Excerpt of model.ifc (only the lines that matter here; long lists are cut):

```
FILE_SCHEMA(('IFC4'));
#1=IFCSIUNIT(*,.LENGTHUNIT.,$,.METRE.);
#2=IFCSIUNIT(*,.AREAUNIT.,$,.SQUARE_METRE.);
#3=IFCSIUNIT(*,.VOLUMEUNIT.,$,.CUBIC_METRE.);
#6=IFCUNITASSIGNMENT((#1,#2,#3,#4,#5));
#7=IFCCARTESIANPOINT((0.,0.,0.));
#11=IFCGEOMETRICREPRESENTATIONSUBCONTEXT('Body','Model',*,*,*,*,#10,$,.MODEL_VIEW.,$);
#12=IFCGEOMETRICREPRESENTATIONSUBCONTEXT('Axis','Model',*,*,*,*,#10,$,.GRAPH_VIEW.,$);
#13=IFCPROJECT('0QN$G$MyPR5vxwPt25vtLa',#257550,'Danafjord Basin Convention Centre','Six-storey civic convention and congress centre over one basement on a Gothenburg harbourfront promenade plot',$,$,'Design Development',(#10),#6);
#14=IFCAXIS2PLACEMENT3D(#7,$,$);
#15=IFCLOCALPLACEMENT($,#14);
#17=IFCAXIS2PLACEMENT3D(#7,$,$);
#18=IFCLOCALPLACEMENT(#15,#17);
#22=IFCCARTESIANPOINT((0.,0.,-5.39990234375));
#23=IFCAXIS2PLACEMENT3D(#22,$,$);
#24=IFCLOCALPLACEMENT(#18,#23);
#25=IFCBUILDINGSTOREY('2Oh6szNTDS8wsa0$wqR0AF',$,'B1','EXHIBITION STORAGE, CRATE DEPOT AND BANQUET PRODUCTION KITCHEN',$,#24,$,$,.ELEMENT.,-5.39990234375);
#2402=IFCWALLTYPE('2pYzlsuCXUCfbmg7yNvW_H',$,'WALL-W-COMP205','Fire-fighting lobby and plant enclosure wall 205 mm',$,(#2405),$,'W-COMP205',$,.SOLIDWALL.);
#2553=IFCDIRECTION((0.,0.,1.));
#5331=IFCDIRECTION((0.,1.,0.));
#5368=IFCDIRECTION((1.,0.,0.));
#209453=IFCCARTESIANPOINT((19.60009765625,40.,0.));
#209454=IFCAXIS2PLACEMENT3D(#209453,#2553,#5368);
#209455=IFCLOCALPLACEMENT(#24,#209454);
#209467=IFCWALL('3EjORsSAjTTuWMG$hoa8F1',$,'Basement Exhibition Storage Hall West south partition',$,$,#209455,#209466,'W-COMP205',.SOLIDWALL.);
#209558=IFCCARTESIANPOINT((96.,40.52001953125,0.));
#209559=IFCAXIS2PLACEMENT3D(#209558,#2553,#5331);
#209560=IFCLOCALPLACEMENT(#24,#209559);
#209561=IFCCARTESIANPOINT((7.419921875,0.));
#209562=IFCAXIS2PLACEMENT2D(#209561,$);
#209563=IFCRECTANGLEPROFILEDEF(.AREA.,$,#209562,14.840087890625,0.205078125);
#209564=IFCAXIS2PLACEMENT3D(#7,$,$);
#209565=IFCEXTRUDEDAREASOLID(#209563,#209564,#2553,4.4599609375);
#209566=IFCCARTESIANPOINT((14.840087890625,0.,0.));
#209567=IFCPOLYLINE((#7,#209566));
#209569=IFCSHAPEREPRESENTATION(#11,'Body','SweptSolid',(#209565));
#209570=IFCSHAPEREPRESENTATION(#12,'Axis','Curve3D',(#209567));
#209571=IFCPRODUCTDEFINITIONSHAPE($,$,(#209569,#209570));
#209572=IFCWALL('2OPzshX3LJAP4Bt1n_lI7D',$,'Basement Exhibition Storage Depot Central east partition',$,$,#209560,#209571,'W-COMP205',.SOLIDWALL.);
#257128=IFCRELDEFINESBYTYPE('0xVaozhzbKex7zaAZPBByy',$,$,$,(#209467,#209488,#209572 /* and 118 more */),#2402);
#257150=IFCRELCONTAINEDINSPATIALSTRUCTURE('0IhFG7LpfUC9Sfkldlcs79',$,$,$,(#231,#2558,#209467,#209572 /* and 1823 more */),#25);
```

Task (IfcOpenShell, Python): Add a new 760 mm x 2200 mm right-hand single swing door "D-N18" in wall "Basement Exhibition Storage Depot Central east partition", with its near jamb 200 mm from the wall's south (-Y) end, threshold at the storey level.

```python
import numpy as np
import ifcopenshell
import ifcopenshell.api.feature
import ifcopenshell.api.geometry
import ifcopenshell.api.root
import ifcopenshell.api.spatial
import ifcopenshell.geom
import ifcopenshell.util.element
import ifcopenshell.util.placement
import ifcopenshell.util.representation
import ifcopenshell.util.shape
import ifcopenshell.util.unit

model = ifcopenshell.open("model.ifc")
unit_scale = ifcopenshell.util.unit.calculate_unit_scale(model)
settings = ifcopenshell.geom.settings()


def volume(element):
    """Net volume in cubic metres, openings subtracted."""
    shape = ifcopenshell.geom.create_shape(settings, element)
    return ifcopenshell.util.shape.get_volume(shape.geometry)


wall = model.by_guid("2OPzshX3LJAP4Bt1n_lI7D")
storey = ifcopenshell.util.element.get_container(wall, ifc_class="IfcBuildingStorey")
context = ifcopenshell.util.representation.get_context(model, "Model", "Body", "MODEL_VIEW")
before = volume(wall)

width, height, from_end, sill = 0.76, 2.2, 0.2, 0.0  # metres

# The wall runs along its own X axis, and the end named is its -X end.
wall_shape = ifcopenshell.geom.create_shape(settings, wall)
x, y, z = ifcopenshell.util.shape.get_vertices(wall_shape.geometry).T
start = x.min() + from_end
face, thickness = float(y.min()), float(y.max() - y.min())
wall_matrix = ifcopenshell.util.placement.get_local_placement(wall.ObjectPlacement)
level = ifcopenshell.util.placement.get_local_placement(storey.ObjectPlacement)[2, 3]


def in_wall(x, y):
    """Placement at x, y metres in the wall's axes, at sill height."""
    matrix = wall_matrix.copy()
    matrix[:, 3] = wall_matrix @ np.array([x / unit_scale, y / unit_scale, 0.0, 1.0])
    matrix[2, 3] = level + sill / unit_scale
    return matrix


# Opening: a box that overshoots both wall faces by 50 mm.
opening = ifcopenshell.api.root.create_entity(model, ifc_class="IfcOpeningElement", predefined_type="OPENING")
box = ifcopenshell.api.geometry.add_wall_representation(
    model, context=context, length=width, height=height, thickness=thickness + 0.1
)
ifcopenshell.api.geometry.assign_representation(model, product=opening, representation=box)
ifcopenshell.api.geometry.edit_object_placement(model, product=opening, matrix=in_wall(start, face - 0.05), is_si=False)
ifcopenshell.api.feature.add_feature(model, feature=opening, element=wall)

door = ifcopenshell.api.root.create_entity(model, ifc_class="IfcDoor", name="D-N18", predefined_type="DOOR")
door.OverallWidth, door.OverallHeight = width / unit_scale, height / unit_scale
door.OperationType = "SINGLE_SWING_RIGHT"
body = ifcopenshell.api.geometry.add_door_representation(
    model,
    context=context,
    overall_width=door.OverallWidth,
    overall_height=door.OverallHeight,
    operation_type="SINGLE_SWING_RIGHT",
    lining_properties={"LiningDepth": thickness / unit_scale, "ThresholdDepth": thickness / unit_scale},
)
ifcopenshell.api.geometry.assign_representation(model, product=door, representation=body)
ifcopenshell.api.spatial.assign_container(model, products=[door], relating_structure=storey)
ifcopenshell.api.feature.add_filling(model, opening=opening, element=door)

# The lining spans the wall, so the door starts at the wall face.
ifcopenshell.api.geometry.edit_object_placement(model, product=door, matrix=in_wall(start, face), is_si=False)

after = volume(wall)

print(f"wall volume {before:.3f} -> {after:.3f} m3")

model.write("model_v2.ifc")
```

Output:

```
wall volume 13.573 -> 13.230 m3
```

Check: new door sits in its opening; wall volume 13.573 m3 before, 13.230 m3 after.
